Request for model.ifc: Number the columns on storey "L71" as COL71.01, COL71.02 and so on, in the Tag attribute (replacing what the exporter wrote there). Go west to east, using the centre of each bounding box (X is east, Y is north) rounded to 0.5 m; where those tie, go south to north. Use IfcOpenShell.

First a look at what the model holds.

```python
import ifcopenshell
import ifcopenshell.util.element
import ifcopenshell.util.placement

model = ifcopenshell.open("model.ifc")
print(model.schema)
storey = next(s for s in model.by_type("IfcBuildingStorey") if s.Name == "L71")
columns = [e for e in ifcopenshell.util.element.get_decomposition(storey) if e.is_a("IfcColumn")]
for e in sorted(columns, key=lambda e: e.id()):
    origin = ifcopenshell.util.placement.get_local_placement(e.ObjectPlacement)[:3, 3]
    print(e.id(), e.Tag, e.Name, origin.round(2) + 0.0, sep=" | ")
```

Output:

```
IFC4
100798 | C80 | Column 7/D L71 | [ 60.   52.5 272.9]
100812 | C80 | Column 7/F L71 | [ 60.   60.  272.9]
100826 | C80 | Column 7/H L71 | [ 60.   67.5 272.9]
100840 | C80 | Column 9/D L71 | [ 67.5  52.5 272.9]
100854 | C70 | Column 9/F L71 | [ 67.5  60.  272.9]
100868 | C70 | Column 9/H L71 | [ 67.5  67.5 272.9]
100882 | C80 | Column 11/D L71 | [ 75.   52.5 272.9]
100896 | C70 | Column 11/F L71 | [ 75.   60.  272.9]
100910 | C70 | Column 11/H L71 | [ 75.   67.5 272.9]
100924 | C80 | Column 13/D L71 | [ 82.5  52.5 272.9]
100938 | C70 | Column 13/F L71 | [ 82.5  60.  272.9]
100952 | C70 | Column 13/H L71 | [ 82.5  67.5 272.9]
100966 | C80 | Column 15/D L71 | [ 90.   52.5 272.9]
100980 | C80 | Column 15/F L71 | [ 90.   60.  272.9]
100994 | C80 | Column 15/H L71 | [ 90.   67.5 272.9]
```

```python
import ifcopenshell
import ifcopenshell.geom
import ifcopenshell.util.element
import ifcopenshell.util.shape

model = ifcopenshell.open("model.ifc")
settings = ifcopenshell.geom.settings()
settings.set("use-world-coords", True)


def centre(element):
    shape = ifcopenshell.geom.create_shape(settings, element)
    return ifcopenshell.util.shape.get_bbox_centroid(shape.geometry)


storey = next(s for s in model.by_type("IfcBuildingStorey") if s.Name == "L71")
columns = [e for e in ifcopenshell.util.element.get_decomposition(storey) if e.is_a("IfcColumn")]

# Insertion points can sit at a corner or the storey origin, so sort by the geometry (in metres).
centres = {e: centre(e) for e in columns}
columns.sort(key=lambda e: (round(centres[e][0] / 0.5), centres[e][1]))

for i, e in enumerate(columns, start=1):
    number = f"COL71.{i:02d}"
    e.Tag = number
    print(e.id(), number)

model.write("model-out.ifc")
```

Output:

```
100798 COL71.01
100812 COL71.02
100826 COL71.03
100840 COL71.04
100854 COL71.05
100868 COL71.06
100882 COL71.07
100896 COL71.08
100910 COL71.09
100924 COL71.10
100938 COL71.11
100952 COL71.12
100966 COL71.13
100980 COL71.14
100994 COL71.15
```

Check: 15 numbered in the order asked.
